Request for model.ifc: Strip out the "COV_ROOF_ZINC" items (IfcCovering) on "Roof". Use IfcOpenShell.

First a look at what the model holds.

```python
import ifcopenshell
import ifcopenshell.util.element

model = ifcopenshell.open("model.ifc")
print(model.schema)
storey = next(s for s in model.by_type("IfcBuildingStorey") if s.Name == "Roof")
coverings = [e for e in ifcopenshell.util.element.get_decomposition(storey) if e.is_a("IfcCovering")]
seen = {}
for e in coverings:
    element_type = ifcopenshell.util.element.get_type(e)
    name = element_type.Name if element_type not in (None, e) else None
    seen[name] = seen.get(name, 0) + 1
for name, count in sorted(seen.items(), key=str):
    print(count, "x", name)
```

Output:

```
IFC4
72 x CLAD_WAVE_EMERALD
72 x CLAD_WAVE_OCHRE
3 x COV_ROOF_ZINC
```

```python
import ifcopenshell
import ifcopenshell.api.root
import ifcopenshell.util.element

model = ifcopenshell.open("model.ifc")

storey = next(s for s in model.by_type("IfcBuildingStorey") if s.Name == "Roof")
coverings = [e for e in ifcopenshell.util.element.get_decomposition(storey) if e.is_a("IfcCovering")]
targets = [e for e in coverings if (t := ifcopenshell.util.element.get_type(e)) not in (None, e) and t.Name == "COV_ROOF_ZINC"]

for e in targets:
    ifcopenshell.api.root.remove_product(model, product=e)
print(len(targets), "removed")

model.write("model_updated.ifc")
```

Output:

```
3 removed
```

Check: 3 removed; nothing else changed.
